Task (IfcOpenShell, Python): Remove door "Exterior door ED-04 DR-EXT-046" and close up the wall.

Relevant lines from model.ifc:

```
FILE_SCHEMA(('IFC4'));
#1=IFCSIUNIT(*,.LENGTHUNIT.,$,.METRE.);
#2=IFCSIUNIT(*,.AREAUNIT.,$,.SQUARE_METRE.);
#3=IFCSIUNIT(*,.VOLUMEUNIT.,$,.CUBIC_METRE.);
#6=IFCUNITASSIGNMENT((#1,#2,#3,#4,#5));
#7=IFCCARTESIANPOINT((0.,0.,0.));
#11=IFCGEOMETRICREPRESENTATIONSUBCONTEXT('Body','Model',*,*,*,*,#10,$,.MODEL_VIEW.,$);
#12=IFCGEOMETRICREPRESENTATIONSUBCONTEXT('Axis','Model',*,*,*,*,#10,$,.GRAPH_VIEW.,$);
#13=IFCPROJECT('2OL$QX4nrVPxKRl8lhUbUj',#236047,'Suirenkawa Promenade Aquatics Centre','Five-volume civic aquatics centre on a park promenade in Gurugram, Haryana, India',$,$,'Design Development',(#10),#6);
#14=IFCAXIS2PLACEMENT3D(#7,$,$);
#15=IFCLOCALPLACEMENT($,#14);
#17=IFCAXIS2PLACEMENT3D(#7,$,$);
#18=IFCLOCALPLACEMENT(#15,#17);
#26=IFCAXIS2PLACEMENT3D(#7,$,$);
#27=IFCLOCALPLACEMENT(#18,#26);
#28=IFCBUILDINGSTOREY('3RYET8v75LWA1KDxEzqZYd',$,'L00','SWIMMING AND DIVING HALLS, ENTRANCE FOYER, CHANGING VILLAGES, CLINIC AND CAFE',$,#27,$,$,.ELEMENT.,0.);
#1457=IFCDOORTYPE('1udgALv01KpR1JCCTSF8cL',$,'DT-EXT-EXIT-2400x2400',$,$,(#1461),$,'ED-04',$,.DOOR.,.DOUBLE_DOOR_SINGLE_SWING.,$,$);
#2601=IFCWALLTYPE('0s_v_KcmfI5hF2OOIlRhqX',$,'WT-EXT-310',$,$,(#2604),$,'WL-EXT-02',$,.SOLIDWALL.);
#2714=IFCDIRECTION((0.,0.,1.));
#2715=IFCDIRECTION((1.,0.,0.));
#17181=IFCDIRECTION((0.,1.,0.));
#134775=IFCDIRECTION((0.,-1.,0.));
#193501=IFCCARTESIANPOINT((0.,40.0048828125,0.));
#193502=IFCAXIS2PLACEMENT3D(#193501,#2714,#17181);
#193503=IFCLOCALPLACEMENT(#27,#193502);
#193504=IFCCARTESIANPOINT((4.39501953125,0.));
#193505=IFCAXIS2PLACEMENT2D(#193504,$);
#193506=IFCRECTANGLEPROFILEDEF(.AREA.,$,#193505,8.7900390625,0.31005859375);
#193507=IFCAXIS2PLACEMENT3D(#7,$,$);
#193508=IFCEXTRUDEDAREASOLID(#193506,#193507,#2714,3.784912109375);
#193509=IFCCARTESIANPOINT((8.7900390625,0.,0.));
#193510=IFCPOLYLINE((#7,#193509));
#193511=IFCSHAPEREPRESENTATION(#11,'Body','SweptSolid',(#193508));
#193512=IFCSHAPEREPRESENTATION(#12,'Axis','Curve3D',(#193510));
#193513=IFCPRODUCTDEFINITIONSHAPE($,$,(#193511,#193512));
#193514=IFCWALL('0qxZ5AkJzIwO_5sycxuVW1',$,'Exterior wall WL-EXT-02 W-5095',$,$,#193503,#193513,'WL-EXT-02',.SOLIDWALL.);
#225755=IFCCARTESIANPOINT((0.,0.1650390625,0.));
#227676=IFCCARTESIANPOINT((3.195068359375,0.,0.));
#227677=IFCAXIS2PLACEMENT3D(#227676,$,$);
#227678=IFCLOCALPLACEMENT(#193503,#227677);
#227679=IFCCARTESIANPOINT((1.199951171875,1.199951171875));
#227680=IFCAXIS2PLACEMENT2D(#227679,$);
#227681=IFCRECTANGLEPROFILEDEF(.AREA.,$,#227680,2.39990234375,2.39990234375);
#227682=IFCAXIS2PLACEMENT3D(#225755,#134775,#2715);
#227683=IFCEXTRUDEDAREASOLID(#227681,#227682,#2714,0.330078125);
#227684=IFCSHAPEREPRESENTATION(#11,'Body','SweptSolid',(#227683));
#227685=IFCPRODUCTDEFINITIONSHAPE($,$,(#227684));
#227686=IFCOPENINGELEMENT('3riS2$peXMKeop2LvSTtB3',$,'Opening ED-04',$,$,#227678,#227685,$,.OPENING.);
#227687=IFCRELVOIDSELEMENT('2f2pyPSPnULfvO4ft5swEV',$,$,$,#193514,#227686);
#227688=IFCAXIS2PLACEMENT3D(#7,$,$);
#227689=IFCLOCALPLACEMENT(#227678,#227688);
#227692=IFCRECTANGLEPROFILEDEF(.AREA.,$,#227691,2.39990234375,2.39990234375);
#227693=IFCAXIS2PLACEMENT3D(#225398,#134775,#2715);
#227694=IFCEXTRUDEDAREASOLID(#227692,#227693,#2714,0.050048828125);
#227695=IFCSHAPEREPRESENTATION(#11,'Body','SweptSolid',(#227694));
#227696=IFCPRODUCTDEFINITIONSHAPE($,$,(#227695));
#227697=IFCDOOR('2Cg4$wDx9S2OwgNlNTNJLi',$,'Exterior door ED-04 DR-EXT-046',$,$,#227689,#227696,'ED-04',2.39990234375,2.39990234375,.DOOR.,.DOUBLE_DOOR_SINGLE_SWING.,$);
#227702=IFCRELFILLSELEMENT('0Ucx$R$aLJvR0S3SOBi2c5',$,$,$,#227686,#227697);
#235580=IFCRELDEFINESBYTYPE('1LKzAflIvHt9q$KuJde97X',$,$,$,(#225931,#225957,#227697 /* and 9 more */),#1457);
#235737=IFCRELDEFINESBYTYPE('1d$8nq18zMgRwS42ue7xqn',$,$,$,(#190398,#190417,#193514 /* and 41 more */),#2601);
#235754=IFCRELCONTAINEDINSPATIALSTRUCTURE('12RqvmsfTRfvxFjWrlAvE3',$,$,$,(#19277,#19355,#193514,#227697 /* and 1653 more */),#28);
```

```python
import ifcopenshell
import ifcopenshell.api.feature
import ifcopenshell.api.root
import ifcopenshell.geom
import ifcopenshell.util.shape

model = ifcopenshell.open("model.ifc")
settings = ifcopenshell.geom.settings()


def volume(element):
    """Net volume in cubic metres, openings subtracted."""
    shape = ifcopenshell.geom.create_shape(settings, element)
    return ifcopenshell.util.shape.get_volume(shape.geometry)


door = model.by_id(227697)
opening = door.FillsVoids[0].RelatingOpeningElement
wall = opening.VoidsElements[0].RelatingBuildingElement
before = volume(wall)

ifcopenshell.api.root.remove_product(model, product=door)
ifcopenshell.api.feature.remove_feature(model, feature=opening)

after = volume(wall)

print(f"wall volume {before:.3f} -> {after:.3f} m3")

model.write("model_v2.ifc")
```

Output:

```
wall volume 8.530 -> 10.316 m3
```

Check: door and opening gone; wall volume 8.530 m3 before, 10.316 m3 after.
